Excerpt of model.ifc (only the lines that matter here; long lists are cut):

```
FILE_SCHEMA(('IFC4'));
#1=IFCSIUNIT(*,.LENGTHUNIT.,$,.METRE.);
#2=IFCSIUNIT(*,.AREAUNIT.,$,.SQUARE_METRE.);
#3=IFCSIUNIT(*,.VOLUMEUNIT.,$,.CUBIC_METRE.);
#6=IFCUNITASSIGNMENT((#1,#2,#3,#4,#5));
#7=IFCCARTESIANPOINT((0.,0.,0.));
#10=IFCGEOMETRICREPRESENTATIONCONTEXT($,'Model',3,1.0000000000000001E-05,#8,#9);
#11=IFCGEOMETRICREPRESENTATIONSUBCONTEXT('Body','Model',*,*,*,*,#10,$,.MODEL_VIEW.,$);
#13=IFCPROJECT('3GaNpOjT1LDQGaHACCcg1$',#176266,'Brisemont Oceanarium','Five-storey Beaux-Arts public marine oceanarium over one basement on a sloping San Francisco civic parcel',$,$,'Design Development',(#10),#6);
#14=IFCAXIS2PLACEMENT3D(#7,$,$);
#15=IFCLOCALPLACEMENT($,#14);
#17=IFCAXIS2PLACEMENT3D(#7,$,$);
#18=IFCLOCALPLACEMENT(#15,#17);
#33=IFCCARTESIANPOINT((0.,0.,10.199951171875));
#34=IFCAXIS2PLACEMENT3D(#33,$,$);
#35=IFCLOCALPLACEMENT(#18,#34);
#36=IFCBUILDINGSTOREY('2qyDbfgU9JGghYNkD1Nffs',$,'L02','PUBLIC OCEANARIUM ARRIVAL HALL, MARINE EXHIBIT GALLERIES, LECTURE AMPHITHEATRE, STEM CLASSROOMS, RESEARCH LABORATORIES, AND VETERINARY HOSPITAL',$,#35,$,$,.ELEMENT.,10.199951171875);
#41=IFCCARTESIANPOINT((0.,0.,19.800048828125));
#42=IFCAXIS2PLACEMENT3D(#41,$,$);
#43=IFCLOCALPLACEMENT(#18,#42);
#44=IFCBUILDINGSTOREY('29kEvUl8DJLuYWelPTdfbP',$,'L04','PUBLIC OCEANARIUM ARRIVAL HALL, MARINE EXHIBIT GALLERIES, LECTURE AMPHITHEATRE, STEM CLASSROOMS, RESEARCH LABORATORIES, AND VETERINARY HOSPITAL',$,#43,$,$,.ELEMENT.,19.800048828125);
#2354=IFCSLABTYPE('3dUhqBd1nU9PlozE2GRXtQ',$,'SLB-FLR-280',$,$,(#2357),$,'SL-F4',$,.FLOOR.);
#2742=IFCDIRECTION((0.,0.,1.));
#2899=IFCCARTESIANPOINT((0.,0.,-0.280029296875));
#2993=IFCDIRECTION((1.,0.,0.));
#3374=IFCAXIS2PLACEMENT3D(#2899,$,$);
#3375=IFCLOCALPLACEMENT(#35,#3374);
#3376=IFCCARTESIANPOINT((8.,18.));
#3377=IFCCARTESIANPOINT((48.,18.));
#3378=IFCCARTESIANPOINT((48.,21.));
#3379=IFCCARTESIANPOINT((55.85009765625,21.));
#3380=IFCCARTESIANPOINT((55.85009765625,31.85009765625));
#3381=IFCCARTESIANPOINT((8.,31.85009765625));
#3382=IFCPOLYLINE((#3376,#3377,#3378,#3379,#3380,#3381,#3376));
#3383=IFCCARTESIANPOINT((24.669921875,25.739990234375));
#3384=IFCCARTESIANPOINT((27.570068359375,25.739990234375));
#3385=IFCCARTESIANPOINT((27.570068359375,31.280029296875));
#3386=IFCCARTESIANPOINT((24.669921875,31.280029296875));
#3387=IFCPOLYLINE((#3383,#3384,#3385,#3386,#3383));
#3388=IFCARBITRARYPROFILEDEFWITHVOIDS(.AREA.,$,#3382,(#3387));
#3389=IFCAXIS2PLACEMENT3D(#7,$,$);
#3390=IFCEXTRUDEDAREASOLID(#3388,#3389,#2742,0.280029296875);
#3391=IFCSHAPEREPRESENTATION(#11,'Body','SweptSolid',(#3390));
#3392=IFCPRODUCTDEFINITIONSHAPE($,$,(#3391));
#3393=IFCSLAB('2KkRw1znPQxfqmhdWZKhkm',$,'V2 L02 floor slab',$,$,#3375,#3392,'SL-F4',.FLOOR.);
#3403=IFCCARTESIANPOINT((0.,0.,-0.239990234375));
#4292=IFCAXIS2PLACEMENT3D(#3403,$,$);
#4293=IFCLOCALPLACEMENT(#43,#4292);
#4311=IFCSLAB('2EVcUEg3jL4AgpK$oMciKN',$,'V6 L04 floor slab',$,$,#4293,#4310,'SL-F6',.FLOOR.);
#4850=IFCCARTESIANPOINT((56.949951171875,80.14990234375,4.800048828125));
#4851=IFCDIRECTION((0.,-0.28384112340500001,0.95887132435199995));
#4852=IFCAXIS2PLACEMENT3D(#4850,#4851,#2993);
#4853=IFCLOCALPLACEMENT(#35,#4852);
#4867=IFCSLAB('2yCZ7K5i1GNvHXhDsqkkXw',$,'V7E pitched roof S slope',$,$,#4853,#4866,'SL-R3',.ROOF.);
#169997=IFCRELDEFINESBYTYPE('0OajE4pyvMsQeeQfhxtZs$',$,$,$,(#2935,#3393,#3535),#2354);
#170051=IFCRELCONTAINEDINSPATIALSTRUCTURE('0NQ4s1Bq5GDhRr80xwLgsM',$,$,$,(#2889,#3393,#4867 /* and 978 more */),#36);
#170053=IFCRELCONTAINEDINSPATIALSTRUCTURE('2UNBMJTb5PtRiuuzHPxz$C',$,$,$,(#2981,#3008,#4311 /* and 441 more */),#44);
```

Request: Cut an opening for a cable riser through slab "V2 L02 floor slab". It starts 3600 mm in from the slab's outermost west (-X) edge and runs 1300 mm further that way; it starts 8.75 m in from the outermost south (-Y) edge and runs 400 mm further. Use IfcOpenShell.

```python
import numpy as np
import ifcopenshell
import ifcopenshell.api.feature
import ifcopenshell.api.geometry
import ifcopenshell.api.root
import ifcopenshell.geom
import ifcopenshell.util.placement
import ifcopenshell.util.representation
import ifcopenshell.util.shape
import ifcopenshell.util.unit

model = ifcopenshell.open("model.ifc")
unit_scale = ifcopenshell.util.unit.calculate_unit_scale(model)
settings = ifcopenshell.geom.settings()


def volume(element):
    """Net volume in cubic metres, openings subtracted."""
    shape = ifcopenshell.geom.create_shape(settings, element)
    return ifcopenshell.util.shape.get_volume(shape.geometry)


slab = model.by_guid("2KkRw1znPQxfqmhdWZKhkm")
before = volume(slab)

# Extent in the slab's own axes, in metres. The edges named are its -X and -Y sides.
slab_shape = ifcopenshell.geom.create_shape(settings, slab)
vertices = ifcopenshell.util.shape.get_vertices(slab_shape.geometry)
x_min, y_min, bottom = vertices.min(axis=0)
top = vertices[:, 2].max()

opening = ifcopenshell.api.root.create_entity(model, ifc_class="IfcOpeningElement", name="Cable riser opening", predefined_type="OPENING")
context = ifcopenshell.util.representation.get_context(model, "Model", "Body", "MODEL_VIEW")
width, depth = 1.3, 0.4
outline = [(0.0, 0.0), (width, 0.0), (width, depth), (0.0, depth), (0.0, 0.0)]
# Overshoot both faces by 50 mm so the cut is clean.
shape = ifcopenshell.api.geometry.add_slab_representation(
    model, context=context, depth=top - bottom + 0.1, polyline=outline
)
ifcopenshell.api.geometry.assign_representation(model, product=opening, representation=shape)

matrix = ifcopenshell.util.placement.get_local_placement(slab.ObjectPlacement)
matrix[:, 3] = matrix @ np.append(np.array([x_min + 3.6, y_min + 8.75, bottom - 0.05]) / unit_scale, 1.0)
ifcopenshell.api.geometry.edit_object_placement(model, product=opening, matrix=matrix, is_si=False)
ifcopenshell.api.feature.add_feature(model, feature=opening, element=slab)

after = volume(slab)

print(f"slab volume {before:.3f} -> {after:.3f} m3")

model.write("model_v2.ifc")
```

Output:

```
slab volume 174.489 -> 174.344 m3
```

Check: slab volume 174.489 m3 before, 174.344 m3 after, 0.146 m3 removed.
